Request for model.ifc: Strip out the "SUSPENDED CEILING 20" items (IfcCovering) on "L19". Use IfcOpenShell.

First a look at what the model holds.

```python
import ifcopenshell
import ifcopenshell.util.element

model = ifcopenshell.open("model.ifc")
print(model.schema)
storey = next(s for s in model.by_type("IfcBuildingStorey") if s.Name == "L19")
coverings = [e for e in ifcopenshell.util.element.get_decomposition(storey) if e.is_a("IfcCovering")]
seen = {}
for e in coverings:
    element_type = ifcopenshell.util.element.get_type(e)
    name = element_type.Name if element_type not in (None, e) else None
    seen[name] = seen.get(name, 0) + 1
for name, count in sorted(seen.items(), key=str):
    print(count, "x", name)
```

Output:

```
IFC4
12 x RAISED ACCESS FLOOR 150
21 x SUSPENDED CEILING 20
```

```python
import ifcopenshell
import ifcopenshell.api.root
import ifcopenshell.util.element

model = ifcopenshell.open("model.ifc")

storey = next(s for s in model.by_type("IfcBuildingStorey") if s.Name == "L19")
coverings = [e for e in ifcopenshell.util.element.get_decomposition(storey) if e.is_a("IfcCovering")]
targets = [e for e in coverings if (t := ifcopenshell.util.element.get_type(e)) not in (None, e) and t.Name == "SUSPENDED CEILING 20"]

for e in targets:
    ifcopenshell.api.root.remove_product(model, product=e)
print(len(targets), "removed")

model.write("model-out.ifc")
```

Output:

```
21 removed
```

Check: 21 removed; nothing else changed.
